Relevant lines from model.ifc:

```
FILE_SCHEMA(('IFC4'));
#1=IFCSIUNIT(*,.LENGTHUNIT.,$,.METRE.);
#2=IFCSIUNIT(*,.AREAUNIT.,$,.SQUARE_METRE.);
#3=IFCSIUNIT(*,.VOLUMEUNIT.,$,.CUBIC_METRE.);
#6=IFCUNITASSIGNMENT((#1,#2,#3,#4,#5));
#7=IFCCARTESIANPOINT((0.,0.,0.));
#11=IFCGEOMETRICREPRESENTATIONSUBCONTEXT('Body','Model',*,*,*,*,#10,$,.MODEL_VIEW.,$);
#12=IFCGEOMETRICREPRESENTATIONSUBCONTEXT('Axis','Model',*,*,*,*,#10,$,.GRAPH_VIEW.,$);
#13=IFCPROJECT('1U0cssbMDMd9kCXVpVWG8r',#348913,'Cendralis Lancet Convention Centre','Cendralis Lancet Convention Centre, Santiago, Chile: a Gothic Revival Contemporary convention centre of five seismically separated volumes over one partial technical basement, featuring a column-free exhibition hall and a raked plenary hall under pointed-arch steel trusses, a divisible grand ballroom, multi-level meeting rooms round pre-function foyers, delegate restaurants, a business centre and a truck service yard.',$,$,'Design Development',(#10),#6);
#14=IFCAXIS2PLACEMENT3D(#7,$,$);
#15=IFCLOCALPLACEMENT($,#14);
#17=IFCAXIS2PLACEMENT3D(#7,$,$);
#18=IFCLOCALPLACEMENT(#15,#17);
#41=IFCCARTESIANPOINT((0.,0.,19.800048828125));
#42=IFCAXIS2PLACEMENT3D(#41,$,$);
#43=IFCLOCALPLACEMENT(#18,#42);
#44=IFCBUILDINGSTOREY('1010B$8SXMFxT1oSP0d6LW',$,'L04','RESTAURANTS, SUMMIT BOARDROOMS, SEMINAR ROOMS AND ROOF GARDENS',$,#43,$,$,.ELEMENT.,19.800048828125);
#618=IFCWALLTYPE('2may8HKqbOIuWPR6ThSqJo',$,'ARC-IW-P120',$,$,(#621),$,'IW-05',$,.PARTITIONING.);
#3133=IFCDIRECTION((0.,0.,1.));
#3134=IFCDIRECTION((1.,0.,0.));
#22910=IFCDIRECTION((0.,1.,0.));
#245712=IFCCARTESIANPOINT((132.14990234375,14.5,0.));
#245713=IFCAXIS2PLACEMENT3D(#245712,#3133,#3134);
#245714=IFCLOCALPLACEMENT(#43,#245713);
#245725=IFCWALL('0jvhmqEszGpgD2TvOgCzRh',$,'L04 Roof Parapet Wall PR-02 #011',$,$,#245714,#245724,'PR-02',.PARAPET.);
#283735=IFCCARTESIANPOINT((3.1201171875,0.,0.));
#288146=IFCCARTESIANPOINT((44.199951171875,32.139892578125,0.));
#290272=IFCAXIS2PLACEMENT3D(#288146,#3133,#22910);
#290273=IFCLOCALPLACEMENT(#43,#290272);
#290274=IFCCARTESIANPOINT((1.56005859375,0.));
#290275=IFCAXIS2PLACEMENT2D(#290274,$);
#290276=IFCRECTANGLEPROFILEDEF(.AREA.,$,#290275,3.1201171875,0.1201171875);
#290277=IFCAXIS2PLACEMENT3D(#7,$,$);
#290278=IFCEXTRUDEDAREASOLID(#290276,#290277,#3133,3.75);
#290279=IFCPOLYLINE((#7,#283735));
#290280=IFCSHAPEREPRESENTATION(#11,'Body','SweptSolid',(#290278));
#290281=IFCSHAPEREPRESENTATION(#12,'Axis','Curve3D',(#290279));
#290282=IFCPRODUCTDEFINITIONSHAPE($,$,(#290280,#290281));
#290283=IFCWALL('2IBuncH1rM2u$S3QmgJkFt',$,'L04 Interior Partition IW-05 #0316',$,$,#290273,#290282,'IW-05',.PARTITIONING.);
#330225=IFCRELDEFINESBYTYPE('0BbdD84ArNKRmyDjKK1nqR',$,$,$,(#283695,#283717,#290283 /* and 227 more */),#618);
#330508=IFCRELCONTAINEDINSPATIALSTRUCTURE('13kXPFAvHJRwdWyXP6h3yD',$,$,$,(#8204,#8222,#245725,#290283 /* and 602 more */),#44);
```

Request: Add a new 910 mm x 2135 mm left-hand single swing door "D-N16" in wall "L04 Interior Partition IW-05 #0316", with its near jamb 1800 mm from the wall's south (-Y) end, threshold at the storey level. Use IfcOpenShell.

```python
import numpy as np
import ifcopenshell
import ifcopenshell.api.feature
import ifcopenshell.api.geometry
import ifcopenshell.api.root
import ifcopenshell.api.spatial
import ifcopenshell.geom
import ifcopenshell.util.element
import ifcopenshell.util.placement
import ifcopenshell.util.representation
import ifcopenshell.util.shape
import ifcopenshell.util.unit

model = ifcopenshell.open("model.ifc")
unit_scale = ifcopenshell.util.unit.calculate_unit_scale(model)
settings = ifcopenshell.geom.settings()


def volume(element):
    """Net volume in cubic metres, openings subtracted."""
    shape = ifcopenshell.geom.create_shape(settings, element)
    return ifcopenshell.util.shape.get_volume(shape.geometry)


wall = model.by_guid("2IBuncH1rM2u$S3QmgJkFt")
storey = ifcopenshell.util.element.get_container(wall, ifc_class="IfcBuildingStorey")
context = ifcopenshell.util.representation.get_context(model, "Model", "Body", "MODEL_VIEW")
before = volume(wall)

width, height, from_end, sill = 0.91, 2.135, 1.8, 0.0  # metres

# The wall runs along its own X axis, and the end named is its -X end.
wall_shape = ifcopenshell.geom.create_shape(settings, wall)
x, y, z = ifcopenshell.util.shape.get_vertices(wall_shape.geometry).T
start = x.min() + from_end
face, thickness = float(y.min()), float(y.max() - y.min())
wall_matrix = ifcopenshell.util.placement.get_local_placement(wall.ObjectPlacement)
level = ifcopenshell.util.placement.get_local_placement(storey.ObjectPlacement)[2, 3]


def in_wall(x, y):
    """Placement at x, y metres in the wall's axes, at sill height."""
    matrix = wall_matrix.copy()
    matrix[:, 3] = wall_matrix @ np.array([x / unit_scale, y / unit_scale, 0.0, 1.0])
    matrix[2, 3] = level + sill / unit_scale
    return matrix


# Opening: a box that overshoots both wall faces by 50 mm.
opening = ifcopenshell.api.root.create_entity(model, ifc_class="IfcOpeningElement", predefined_type="OPENING")
box = ifcopenshell.api.geometry.add_wall_representation(
    model, context=context, length=width, height=height, thickness=thickness + 0.1
)
ifcopenshell.api.geometry.assign_representation(model, product=opening, representation=box)
ifcopenshell.api.geometry.edit_object_placement(model, product=opening, matrix=in_wall(start, face - 0.05), is_si=False)
ifcopenshell.api.feature.add_feature(model, feature=opening, element=wall)

door = ifcopenshell.api.root.create_entity(model, ifc_class="IfcDoor", name="D-N16", predefined_type="DOOR")
door.OverallWidth, door.OverallHeight = width / unit_scale, height / unit_scale
door.OperationType = "SINGLE_SWING_LEFT"
body = ifcopenshell.api.geometry.add_door_representation(
    model,
    context=context,
    overall_width=door.OverallWidth,
    overall_height=door.OverallHeight,
    operation_type="SINGLE_SWING_LEFT",
    lining_properties={"LiningDepth": thickness / unit_scale, "ThresholdDepth": thickness / unit_scale},
)
ifcopenshell.api.geometry.assign_representation(model, product=door, representation=body)
ifcopenshell.api.spatial.assign_container(model, products=[door], relating_structure=storey)
ifcopenshell.api.feature.add_filling(model, opening=opening, element=door)

# The lining spans the wall, so the door starts at the wall face.
ifcopenshell.api.geometry.edit_object_placement(model, product=door, matrix=in_wall(start, face), is_si=False)

after = volume(wall)

print(f"wall volume {before:.3f} -> {after:.3f} m3")

model.write("model-out.ifc")
```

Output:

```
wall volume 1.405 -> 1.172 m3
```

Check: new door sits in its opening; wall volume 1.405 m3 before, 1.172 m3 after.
